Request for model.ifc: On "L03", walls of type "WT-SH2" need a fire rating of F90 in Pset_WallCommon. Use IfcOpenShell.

First a look at what the model holds.

```python
import ifcopenshell
import ifcopenshell.util.element

model = ifcopenshell.open("model.ifc")
print(model.schema)
storey = next(s for s in model.by_type("IfcBuildingStorey") if s.Name == "L03")
walls = [e for e in ifcopenshell.util.element.get_decomposition(storey) if e.is_a("IfcWall")]
seen = {}
for e in walls:
    element_type = ifcopenshell.util.element.get_type(e)
    key = (element_type.Name if element_type != e and element_type else None, ifcopenshell.util.element.get_pset(e, "Pset_WallCommon", "FireRating"))
    seen[key] = seen.get(key, 0) + 1
for (name, value), count in sorted(seen.items(), key=str):
    print(count, "x", name, "|", value)
```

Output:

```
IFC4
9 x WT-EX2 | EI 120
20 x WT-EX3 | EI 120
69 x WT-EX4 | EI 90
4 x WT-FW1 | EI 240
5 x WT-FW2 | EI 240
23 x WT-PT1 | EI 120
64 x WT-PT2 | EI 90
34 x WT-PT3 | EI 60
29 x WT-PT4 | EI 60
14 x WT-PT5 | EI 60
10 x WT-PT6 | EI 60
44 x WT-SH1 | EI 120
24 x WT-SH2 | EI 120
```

```python
import ifcopenshell
import ifcopenshell.api.pset
import ifcopenshell.util.element

model = ifcopenshell.open("model.ifc")

storey = next(s for s in model.by_type("IfcBuildingStorey") if s.Name == "L03")
walls = [e for e in ifcopenshell.util.element.get_decomposition(storey) if e.is_a("IfcWall")]

count = 0
for e in walls:
    element_type = ifcopenshell.util.element.get_type(e)
    if element_type in (None, e) or element_type.Name != "WT-SH2":
        continue
    # add_pset returns the element's existing set when there is one.
    pset = ifcopenshell.api.pset.add_pset(model, product=e, name="Pset_WallCommon")
    ifcopenshell.api.pset.edit_pset(model, pset=pset, properties={"FireRating": "F90"})
    count += 1

print(count, "walls updated")

model.write("model-out.ifc")
```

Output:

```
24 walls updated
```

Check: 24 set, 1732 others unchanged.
